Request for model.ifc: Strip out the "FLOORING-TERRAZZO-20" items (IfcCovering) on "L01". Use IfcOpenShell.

First a look at what the model holds.

```python
import ifcopenshell
import ifcopenshell.util.element

model = ifcopenshell.open("model.ifc")
print(model.schema)
storey = next(s for s in model.by_type("IfcBuildingStorey") if s.Name == "L01")
coverings = [e for e in ifcopenshell.util.element.get_decomposition(storey) if e.is_a("IfcCovering")]
seen = {}
for e in coverings:
    element_type = ifcopenshell.util.element.get_type(e)
    name = element_type.Name if element_type not in (None, e) else None
    seen[name] = seen.get(name, 0) + 1
for name, count in sorted(seen.items(), key=str):
    print(count, "x", name)
```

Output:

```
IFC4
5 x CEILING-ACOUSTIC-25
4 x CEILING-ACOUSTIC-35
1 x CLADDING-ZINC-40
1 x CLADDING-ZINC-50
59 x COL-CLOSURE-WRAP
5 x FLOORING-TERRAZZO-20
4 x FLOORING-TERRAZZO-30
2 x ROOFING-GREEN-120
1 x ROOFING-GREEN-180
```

```python
import ifcopenshell
import ifcopenshell.api.root
import ifcopenshell.util.element

model = ifcopenshell.open("model.ifc")

storey = next(s for s in model.by_type("IfcBuildingStorey") if s.Name == "L01")
coverings = [e for e in ifcopenshell.util.element.get_decomposition(storey) if e.is_a("IfcCovering")]
targets = [e for e in coverings if (t := ifcopenshell.util.element.get_type(e)) not in (None, e) and t.Name == "FLOORING-TERRAZZO-20"]

for e in targets:
    ifcopenshell.api.root.remove_product(model, product=e)
print(len(targets), "removed")

model.write("model_updated.ifc")
```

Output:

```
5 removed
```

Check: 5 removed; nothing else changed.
